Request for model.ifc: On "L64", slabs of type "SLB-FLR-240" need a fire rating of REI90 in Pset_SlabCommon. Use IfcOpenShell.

First a look at what the model holds.

```python
import ifcopenshell
import ifcopenshell.util.element

model = ifcopenshell.open("model.ifc")
print(model.schema)
storey = next(s for s in model.by_type("IfcBuildingStorey") if s.Name == "L64")
slabs = [e for e in ifcopenshell.util.element.get_decomposition(storey) if e.is_a("IfcSlab")]
seen = {}
for e in slabs:
    element_type = ifcopenshell.util.element.get_type(e)
    key = (element_type.Name if element_type != e and element_type else None, ifcopenshell.util.element.get_pset(e, "Pset_SlabCommon", "FireRating"))
    seen[key] = seen.get(key, 0) + 1
for (name, value), count in sorted(seen.items(), key=str):
    print(count, "x", name, "|", value)
```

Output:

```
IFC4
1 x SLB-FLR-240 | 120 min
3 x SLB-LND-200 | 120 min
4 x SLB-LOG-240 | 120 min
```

```python
import ifcopenshell
import ifcopenshell.api.pset
import ifcopenshell.util.element

model = ifcopenshell.open("model.ifc")

storey = next(s for s in model.by_type("IfcBuildingStorey") if s.Name == "L64")
slabs = [e for e in ifcopenshell.util.element.get_decomposition(storey) if e.is_a("IfcSlab")]

count = 0
for e in slabs:
    element_type = ifcopenshell.util.element.get_type(e)
    if element_type in (None, e) or element_type.Name != "SLB-FLR-240":
        continue
    # add_pset returns the element's existing set when there is one.
    pset = ifcopenshell.api.pset.add_pset(model, product=e, name="Pset_SlabCommon")
    ifcopenshell.api.pset.edit_pset(model, pset=pset, properties={"FireRating": "REI90"})
    count += 1

print(count, "slabs updated")

model.write("model_updated.ifc")
```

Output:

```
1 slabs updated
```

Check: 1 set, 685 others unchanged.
